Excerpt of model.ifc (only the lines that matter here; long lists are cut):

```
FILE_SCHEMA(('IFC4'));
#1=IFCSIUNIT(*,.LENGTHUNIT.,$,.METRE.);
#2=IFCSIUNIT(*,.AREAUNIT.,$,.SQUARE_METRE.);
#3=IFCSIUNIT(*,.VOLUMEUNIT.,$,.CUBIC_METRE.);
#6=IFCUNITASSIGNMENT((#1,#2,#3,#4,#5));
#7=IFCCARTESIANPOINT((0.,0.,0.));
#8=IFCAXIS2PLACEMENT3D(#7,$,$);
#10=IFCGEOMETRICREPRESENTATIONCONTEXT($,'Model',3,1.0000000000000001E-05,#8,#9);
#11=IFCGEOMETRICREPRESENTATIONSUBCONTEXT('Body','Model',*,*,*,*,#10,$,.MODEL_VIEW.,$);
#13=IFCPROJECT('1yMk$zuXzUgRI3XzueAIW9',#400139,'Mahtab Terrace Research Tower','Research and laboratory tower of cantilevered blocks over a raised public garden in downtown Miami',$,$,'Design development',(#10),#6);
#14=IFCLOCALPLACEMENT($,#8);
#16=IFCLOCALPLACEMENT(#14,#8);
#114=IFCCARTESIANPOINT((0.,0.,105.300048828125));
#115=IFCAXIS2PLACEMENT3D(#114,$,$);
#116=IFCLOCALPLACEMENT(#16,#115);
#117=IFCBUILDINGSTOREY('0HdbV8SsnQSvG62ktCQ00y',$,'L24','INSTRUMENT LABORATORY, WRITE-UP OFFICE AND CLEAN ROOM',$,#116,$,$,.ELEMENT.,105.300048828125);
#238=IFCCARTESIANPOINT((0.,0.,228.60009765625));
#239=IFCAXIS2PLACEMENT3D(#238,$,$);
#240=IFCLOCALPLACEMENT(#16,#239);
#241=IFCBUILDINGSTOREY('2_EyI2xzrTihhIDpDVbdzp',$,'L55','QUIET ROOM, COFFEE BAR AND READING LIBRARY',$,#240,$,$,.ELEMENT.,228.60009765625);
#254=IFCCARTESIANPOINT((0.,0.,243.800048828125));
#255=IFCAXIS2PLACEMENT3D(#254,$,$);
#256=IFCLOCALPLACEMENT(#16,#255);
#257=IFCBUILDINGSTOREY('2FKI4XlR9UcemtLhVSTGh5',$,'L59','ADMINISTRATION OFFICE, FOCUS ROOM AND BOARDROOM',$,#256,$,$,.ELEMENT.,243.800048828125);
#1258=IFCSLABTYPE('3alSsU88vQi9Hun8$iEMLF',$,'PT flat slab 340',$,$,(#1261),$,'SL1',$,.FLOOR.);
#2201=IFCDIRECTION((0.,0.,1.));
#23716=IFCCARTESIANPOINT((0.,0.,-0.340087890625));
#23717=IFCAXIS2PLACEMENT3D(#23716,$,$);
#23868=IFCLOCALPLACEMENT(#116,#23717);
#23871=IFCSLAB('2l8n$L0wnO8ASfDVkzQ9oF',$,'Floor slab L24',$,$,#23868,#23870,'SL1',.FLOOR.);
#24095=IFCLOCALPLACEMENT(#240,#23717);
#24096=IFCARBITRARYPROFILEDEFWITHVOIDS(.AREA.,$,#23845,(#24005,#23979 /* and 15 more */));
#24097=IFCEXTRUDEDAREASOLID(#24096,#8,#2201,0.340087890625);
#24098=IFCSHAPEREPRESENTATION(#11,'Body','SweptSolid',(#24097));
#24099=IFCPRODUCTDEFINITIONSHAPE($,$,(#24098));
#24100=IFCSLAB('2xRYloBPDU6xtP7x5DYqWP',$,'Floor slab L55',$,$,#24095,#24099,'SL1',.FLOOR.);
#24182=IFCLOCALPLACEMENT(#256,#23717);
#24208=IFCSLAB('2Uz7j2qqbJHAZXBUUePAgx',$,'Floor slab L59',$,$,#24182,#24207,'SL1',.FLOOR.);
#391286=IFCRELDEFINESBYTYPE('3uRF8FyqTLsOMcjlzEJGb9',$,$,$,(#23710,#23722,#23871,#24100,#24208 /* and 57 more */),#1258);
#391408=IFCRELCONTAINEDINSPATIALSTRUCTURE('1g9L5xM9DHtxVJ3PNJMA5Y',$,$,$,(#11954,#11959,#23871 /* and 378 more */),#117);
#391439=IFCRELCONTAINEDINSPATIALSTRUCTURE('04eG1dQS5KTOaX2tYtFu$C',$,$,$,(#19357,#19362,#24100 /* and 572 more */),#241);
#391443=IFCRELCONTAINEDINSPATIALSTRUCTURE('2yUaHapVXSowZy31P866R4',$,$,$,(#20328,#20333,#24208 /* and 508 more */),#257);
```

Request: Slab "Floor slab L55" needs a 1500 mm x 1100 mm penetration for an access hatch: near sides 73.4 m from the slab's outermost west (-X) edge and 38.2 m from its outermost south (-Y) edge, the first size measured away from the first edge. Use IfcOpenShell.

```python
import numpy as np
import ifcopenshell
import ifcopenshell.api.feature
import ifcopenshell.api.geometry
import ifcopenshell.api.root
import ifcopenshell.geom
import ifcopenshell.util.placement
import ifcopenshell.util.representation
import ifcopenshell.util.shape
import ifcopenshell.util.unit

model = ifcopenshell.open("model.ifc")
unit_scale = ifcopenshell.util.unit.calculate_unit_scale(model)
settings = ifcopenshell.geom.settings()


def volume(element):
    """Net volume in cubic metres, openings subtracted."""
    shape = ifcopenshell.geom.create_shape(settings, element)
    return ifcopenshell.util.shape.get_volume(shape.geometry)


slab = model.by_id(24100)
before = volume(slab)

# Extent in the slab's own axes, in metres. The edges named are its -X and -Y sides.
slab_shape = ifcopenshell.geom.create_shape(settings, slab)
vertices = ifcopenshell.util.shape.get_vertices(slab_shape.geometry)
x_min, y_min, bottom = vertices.min(axis=0)
top = vertices[:, 2].max()

opening = ifcopenshell.api.root.create_entity(model, ifc_class="IfcOpeningElement", name="Access hatch opening", predefined_type="OPENING")
context = ifcopenshell.util.representation.get_context(model, "Model", "Body", "MODEL_VIEW")
width, depth = 1.5, 1.1
outline = [(0.0, 0.0), (width, 0.0), (width, depth), (0.0, depth), (0.0, 0.0)]
# Overshoot both faces by 50 mm so the cut is clean.
shape = ifcopenshell.api.geometry.add_slab_representation(
    model, context=context, depth=top - bottom + 0.1, polyline=outline
)
ifcopenshell.api.geometry.assign_representation(model, product=opening, representation=shape)

matrix = ifcopenshell.util.placement.get_local_placement(slab.ObjectPlacement)
matrix[:, 3] = matrix @ np.append(np.array([x_min + 73.4, y_min + 38.2, bottom - 0.05]) / unit_scale, 1.0)
ifcopenshell.api.geometry.edit_object_placement(model, product=opening, matrix=matrix, is_si=False)
ifcopenshell.api.feature.add_feature(model, feature=opening, element=slab)

after = volume(slab)

print(f"slab volume {before:.3f} -> {after:.3f} m3")

model.write("model_updated.ifc")
```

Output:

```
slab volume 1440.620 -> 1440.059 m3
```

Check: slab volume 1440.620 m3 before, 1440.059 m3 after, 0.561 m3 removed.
